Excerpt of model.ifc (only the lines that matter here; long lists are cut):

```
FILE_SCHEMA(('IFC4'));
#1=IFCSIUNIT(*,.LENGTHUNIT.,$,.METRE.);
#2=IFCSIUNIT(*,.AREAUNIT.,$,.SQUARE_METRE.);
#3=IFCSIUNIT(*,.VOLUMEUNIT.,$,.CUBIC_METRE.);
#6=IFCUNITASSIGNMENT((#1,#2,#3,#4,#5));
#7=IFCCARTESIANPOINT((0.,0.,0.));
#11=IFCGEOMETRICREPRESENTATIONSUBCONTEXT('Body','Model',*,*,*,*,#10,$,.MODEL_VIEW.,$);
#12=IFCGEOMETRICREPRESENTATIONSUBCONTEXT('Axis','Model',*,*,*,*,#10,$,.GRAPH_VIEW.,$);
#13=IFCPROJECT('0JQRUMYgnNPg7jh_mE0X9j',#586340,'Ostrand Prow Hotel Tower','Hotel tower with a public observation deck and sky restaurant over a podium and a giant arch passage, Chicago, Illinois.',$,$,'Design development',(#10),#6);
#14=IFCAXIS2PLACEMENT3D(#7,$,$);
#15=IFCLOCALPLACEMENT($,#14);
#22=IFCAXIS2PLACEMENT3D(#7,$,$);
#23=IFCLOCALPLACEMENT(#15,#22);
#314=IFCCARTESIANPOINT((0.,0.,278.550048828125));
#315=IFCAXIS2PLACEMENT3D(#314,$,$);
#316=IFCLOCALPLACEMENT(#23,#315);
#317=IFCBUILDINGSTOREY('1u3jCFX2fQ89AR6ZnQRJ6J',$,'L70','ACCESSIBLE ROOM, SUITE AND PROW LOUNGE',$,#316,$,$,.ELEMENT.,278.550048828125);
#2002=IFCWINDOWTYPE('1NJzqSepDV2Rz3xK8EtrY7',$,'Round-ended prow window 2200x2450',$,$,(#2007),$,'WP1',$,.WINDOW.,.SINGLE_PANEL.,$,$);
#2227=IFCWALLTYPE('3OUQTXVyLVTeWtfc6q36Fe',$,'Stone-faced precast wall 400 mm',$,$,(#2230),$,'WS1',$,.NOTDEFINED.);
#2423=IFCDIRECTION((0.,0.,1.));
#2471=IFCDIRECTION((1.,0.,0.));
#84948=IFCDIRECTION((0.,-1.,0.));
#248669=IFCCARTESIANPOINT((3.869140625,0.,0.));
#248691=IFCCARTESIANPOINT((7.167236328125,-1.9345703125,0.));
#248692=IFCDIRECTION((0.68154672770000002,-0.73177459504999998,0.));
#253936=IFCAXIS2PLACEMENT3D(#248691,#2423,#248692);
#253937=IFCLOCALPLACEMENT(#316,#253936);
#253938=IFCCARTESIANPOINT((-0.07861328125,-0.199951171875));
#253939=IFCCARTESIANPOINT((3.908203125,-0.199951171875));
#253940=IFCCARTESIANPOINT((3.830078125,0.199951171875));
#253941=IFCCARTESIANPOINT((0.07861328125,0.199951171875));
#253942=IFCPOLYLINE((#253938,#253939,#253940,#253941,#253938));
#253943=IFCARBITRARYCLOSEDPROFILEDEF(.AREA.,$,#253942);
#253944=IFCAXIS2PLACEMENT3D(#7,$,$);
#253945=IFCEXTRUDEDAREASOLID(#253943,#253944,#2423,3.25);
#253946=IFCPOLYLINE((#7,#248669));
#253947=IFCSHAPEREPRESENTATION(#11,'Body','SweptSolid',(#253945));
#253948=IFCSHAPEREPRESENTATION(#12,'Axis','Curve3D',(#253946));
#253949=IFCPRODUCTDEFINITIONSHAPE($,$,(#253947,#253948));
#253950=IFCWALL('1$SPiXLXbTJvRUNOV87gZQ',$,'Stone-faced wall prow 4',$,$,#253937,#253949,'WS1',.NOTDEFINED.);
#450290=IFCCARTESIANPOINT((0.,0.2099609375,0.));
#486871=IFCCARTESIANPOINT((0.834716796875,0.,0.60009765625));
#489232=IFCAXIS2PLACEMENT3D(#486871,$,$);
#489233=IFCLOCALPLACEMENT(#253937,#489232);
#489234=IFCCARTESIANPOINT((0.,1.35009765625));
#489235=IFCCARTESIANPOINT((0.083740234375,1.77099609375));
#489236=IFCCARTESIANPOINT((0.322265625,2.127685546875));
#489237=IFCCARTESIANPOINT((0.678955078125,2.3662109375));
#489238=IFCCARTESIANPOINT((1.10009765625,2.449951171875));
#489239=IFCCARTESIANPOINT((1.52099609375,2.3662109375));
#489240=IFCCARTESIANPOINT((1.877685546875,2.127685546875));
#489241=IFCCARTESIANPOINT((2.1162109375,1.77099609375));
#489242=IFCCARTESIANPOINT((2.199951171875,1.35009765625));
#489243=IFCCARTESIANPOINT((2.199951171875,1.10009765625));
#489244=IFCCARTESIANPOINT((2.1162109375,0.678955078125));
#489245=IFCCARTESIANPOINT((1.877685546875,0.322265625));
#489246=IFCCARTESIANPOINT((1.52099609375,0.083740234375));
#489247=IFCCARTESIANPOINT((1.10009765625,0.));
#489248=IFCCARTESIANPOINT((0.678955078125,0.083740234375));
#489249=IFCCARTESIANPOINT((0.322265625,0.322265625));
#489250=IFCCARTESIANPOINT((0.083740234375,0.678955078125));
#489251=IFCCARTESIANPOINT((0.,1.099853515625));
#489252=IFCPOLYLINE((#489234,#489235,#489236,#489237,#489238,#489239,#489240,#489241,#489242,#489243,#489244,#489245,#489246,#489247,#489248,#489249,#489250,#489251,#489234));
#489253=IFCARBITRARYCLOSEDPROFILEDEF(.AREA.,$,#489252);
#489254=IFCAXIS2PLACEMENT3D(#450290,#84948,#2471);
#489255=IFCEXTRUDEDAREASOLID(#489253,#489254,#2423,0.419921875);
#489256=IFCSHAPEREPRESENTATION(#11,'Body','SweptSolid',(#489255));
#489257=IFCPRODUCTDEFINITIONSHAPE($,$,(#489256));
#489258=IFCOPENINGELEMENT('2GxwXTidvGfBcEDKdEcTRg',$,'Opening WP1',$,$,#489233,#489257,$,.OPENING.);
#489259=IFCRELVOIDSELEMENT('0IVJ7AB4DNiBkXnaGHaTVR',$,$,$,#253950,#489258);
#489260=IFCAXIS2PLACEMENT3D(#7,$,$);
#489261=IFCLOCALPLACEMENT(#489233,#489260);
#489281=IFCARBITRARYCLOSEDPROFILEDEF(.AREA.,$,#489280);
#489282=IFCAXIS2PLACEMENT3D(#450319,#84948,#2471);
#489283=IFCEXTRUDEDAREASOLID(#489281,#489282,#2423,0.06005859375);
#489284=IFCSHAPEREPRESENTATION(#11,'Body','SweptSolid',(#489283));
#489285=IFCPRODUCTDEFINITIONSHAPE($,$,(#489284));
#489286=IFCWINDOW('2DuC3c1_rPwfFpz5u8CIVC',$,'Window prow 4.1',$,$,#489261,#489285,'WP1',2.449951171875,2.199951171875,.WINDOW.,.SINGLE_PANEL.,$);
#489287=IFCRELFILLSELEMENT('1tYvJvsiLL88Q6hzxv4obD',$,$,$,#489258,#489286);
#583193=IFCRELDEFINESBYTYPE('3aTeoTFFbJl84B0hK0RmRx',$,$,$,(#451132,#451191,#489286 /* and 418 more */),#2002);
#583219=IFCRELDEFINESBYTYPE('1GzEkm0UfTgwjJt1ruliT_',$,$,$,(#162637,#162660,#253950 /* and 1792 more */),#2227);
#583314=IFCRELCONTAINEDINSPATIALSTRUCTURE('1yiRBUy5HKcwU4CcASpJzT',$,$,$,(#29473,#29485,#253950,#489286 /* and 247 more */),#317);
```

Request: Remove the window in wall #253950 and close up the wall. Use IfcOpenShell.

```python
import ifcopenshell
import ifcopenshell.api.feature
import ifcopenshell.api.root
import ifcopenshell.geom
import ifcopenshell.util.shape

model = ifcopenshell.open("model.ifc")
settings = ifcopenshell.geom.settings()


def volume(element):
    """Net volume in cubic metres, openings subtracted."""
    shape = ifcopenshell.geom.create_shape(settings, element)
    return ifcopenshell.util.shape.get_volume(shape.geometry)


window = model.by_guid("2DuC3c1_rPwfFpz5u8CIVC")
opening = window.FillsVoids[0].RelatingOpeningElement
wall = opening.VoidsElements[0].RelatingBuildingElement
before = volume(wall)

ifcopenshell.api.root.remove_product(model, product=window)
ifcopenshell.api.feature.remove_feature(model, feature=opening)

after = volume(wall)

print(f"wall volume {before:.3f} -> {after:.3f} m3")

model.write("model_edited.ifc")
```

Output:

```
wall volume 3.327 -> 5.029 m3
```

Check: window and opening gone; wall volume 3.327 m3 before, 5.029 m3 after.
